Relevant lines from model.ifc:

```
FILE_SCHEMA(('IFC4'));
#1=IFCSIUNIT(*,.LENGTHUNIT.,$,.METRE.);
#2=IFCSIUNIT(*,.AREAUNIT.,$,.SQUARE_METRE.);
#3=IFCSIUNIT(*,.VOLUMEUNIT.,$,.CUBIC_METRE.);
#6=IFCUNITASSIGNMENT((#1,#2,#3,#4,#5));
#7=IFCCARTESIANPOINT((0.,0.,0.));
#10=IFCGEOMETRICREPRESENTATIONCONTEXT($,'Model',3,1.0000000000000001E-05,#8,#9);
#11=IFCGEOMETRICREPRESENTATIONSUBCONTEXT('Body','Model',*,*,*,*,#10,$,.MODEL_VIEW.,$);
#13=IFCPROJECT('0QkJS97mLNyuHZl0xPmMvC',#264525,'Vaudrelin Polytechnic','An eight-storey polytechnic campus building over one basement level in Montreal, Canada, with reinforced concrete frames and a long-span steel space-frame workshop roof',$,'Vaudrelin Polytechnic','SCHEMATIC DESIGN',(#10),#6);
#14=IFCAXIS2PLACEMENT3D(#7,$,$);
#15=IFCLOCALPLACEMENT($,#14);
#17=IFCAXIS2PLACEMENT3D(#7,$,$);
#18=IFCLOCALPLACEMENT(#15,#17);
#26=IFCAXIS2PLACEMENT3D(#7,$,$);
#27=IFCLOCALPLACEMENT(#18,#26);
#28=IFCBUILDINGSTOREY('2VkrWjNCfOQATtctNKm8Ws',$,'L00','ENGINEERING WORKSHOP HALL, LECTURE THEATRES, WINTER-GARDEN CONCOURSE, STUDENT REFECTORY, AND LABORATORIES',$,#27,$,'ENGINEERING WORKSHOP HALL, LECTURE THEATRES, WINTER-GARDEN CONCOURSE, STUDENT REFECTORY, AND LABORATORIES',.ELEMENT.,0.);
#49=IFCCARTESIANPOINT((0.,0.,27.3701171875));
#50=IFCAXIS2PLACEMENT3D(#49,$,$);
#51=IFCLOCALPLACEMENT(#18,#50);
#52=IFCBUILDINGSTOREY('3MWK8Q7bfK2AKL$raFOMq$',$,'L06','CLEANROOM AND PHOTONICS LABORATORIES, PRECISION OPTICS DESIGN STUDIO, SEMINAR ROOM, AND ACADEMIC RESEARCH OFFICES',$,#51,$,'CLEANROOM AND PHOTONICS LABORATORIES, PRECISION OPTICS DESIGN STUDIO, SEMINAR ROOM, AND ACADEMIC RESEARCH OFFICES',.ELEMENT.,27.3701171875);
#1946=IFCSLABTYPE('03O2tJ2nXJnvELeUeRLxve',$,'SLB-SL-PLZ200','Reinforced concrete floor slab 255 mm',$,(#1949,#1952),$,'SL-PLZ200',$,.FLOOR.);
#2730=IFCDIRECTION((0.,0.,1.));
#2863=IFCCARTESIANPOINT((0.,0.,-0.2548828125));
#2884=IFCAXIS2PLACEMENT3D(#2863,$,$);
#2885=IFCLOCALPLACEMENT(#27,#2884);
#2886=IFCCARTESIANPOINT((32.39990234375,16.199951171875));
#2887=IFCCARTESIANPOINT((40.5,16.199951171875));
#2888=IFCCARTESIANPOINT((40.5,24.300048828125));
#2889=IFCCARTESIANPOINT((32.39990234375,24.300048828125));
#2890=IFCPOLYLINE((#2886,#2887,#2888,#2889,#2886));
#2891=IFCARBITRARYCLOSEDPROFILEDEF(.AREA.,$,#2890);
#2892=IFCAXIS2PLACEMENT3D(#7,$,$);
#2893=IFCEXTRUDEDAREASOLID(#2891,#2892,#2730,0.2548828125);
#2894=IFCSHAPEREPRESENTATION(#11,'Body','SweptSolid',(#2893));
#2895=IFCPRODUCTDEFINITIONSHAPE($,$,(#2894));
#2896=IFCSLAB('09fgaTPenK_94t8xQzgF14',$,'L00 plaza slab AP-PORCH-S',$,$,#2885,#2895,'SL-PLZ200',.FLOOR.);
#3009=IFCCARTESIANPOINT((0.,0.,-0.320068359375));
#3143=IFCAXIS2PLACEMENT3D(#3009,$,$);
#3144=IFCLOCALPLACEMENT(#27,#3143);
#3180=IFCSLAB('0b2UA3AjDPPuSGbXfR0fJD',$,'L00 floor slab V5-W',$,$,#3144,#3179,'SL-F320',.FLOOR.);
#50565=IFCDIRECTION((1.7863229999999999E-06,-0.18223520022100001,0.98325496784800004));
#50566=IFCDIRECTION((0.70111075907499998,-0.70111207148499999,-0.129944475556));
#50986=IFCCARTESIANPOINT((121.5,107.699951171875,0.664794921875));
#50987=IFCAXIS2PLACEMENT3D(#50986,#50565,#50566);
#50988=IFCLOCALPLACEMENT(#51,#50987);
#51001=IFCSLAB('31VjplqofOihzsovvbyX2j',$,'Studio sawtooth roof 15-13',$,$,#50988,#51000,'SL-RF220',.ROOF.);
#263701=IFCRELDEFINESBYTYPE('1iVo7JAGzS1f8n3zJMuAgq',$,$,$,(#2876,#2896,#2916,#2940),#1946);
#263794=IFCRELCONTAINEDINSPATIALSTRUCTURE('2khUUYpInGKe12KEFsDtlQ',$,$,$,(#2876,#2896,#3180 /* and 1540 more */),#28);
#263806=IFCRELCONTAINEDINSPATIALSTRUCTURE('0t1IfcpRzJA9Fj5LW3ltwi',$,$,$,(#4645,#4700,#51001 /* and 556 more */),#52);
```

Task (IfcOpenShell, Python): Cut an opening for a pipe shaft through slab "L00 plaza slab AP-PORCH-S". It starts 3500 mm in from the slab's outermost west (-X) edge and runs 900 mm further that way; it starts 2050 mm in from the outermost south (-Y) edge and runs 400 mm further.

```python
import numpy as np
import ifcopenshell
import ifcopenshell.api.feature
import ifcopenshell.api.geometry
import ifcopenshell.api.root
import ifcopenshell.geom
import ifcopenshell.util.placement
import ifcopenshell.util.representation
import ifcopenshell.util.shape
import ifcopenshell.util.unit

model = ifcopenshell.open("model.ifc")
unit_scale = ifcopenshell.util.unit.calculate_unit_scale(model)
settings = ifcopenshell.geom.settings()


def volume(element):
    """Net volume in cubic metres, openings subtracted."""
    shape = ifcopenshell.geom.create_shape(settings, element)
    return ifcopenshell.util.shape.get_volume(shape.geometry)


slab = model.by_id(2896)
before = volume(slab)

# Extent in the slab's own axes, in metres. The edges named are its -X and -Y sides.
slab_shape = ifcopenshell.geom.create_shape(settings, slab)
vertices = ifcopenshell.util.shape.get_vertices(slab_shape.geometry)
x_min, y_min, bottom = vertices.min(axis=0)
top = vertices[:, 2].max()

opening = ifcopenshell.api.root.create_entity(model, ifc_class="IfcOpeningElement", name="Pipe shaft opening", predefined_type="OPENING")
context = ifcopenshell.util.representation.get_context(model, "Model", "Body", "MODEL_VIEW")
width, depth = 0.9, 0.4
outline = [(0.0, 0.0), (width, 0.0), (width, depth), (0.0, depth), (0.0, 0.0)]
# Overshoot both faces by 50 mm so the cut is clean.
shape = ifcopenshell.api.geometry.add_slab_representation(
    model, context=context, depth=top - bottom + 0.1, polyline=outline
)
ifcopenshell.api.geometry.assign_representation(model, product=opening, representation=shape)

matrix = ifcopenshell.util.placement.get_local_placement(slab.ObjectPlacement)
matrix[:, 3] = matrix @ np.append(np.array([x_min + 3.5, y_min + 2.05, bottom - 0.05]) / unit_scale, 1.0)
ifcopenshell.api.geometry.edit_object_placement(model, product=opening, matrix=matrix, is_si=False)
ifcopenshell.api.feature.add_feature(model, feature=opening, element=slab)

after = volume(slab)

print(f"slab volume {before:.3f} -> {after:.3f} m3")

model.write("model_v2.ifc")
```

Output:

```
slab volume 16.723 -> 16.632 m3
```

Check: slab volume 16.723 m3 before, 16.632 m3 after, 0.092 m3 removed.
